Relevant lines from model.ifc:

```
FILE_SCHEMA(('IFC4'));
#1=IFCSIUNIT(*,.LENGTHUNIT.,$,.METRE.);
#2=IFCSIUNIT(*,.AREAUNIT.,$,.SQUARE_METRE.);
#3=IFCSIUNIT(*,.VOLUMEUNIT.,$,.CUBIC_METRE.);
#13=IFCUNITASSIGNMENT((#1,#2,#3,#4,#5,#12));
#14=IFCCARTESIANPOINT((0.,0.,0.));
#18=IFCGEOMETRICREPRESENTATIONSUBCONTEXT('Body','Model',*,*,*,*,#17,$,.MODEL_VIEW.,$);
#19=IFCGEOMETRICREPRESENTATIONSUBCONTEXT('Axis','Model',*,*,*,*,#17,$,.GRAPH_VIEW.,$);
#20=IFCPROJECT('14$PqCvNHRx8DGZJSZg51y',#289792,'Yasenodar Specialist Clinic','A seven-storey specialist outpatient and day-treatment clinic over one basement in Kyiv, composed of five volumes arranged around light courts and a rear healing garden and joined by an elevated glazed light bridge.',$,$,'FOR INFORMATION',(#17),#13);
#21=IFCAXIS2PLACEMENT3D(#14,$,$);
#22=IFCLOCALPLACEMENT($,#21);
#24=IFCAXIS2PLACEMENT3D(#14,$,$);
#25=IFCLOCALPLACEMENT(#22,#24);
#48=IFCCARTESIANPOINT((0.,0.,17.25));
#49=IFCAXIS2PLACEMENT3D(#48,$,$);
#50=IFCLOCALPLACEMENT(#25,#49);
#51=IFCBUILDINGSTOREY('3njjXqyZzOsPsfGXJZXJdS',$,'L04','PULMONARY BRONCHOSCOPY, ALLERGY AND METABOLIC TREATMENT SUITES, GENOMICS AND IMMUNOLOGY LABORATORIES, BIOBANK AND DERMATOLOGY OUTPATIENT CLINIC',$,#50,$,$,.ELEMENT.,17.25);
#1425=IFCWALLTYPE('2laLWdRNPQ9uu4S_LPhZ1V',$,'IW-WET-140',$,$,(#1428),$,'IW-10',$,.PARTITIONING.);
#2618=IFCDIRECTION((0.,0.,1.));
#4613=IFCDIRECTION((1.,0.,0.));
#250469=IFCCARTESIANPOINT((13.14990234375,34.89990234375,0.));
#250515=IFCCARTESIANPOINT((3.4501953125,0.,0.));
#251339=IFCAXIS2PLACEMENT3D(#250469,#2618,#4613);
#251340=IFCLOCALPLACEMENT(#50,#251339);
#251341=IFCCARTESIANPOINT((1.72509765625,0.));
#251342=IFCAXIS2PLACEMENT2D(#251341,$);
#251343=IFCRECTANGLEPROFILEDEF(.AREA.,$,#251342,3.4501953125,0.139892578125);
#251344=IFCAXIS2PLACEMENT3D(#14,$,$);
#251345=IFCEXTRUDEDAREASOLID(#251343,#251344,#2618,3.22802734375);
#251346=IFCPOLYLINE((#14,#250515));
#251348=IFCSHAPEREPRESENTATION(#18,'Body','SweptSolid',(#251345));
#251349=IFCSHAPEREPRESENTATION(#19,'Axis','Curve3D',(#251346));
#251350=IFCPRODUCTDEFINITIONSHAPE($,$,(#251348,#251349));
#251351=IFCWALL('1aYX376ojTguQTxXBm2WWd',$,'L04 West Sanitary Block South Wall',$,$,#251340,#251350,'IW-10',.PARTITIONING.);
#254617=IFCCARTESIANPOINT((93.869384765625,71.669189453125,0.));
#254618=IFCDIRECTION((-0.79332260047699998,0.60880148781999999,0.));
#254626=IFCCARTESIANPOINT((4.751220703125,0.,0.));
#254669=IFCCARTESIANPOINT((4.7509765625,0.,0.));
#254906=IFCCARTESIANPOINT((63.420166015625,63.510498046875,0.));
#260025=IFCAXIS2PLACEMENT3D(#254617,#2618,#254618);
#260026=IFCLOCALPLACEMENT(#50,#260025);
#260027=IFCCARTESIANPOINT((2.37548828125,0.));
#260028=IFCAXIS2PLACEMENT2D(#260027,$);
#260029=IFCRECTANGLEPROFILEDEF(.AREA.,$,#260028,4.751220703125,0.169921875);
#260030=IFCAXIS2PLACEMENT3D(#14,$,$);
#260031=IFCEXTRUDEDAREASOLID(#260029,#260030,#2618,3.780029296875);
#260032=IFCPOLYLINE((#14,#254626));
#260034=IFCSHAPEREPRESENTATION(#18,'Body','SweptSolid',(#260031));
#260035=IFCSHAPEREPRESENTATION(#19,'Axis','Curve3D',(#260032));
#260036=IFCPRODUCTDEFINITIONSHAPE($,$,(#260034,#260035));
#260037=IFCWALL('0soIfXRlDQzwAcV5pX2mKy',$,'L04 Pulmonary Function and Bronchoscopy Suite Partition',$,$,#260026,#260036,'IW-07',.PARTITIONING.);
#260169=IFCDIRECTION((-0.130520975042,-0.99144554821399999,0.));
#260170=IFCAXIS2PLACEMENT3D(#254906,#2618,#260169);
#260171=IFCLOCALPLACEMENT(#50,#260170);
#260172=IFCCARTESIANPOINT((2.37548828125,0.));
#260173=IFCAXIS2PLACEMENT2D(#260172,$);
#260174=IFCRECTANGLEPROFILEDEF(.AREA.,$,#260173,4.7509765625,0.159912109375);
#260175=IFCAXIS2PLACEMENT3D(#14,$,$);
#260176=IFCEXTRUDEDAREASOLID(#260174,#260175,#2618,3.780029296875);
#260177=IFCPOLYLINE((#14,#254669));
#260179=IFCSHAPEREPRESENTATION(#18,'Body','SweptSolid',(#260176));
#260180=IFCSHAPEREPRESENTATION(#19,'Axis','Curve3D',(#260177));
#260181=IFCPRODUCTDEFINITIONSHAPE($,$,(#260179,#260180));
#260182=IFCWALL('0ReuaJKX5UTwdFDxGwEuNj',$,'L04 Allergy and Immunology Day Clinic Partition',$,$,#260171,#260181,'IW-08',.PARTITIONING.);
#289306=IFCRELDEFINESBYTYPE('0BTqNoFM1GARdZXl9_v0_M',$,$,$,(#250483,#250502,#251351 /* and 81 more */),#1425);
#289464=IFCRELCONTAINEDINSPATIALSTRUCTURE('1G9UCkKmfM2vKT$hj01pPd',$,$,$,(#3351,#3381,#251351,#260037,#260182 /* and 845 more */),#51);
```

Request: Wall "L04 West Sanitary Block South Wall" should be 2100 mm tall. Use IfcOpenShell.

```python
import ifcopenshell
import ifcopenshell.geom
import ifcopenshell.util.representation
import ifcopenshell.util.shape
import ifcopenshell.util.unit

model = ifcopenshell.open("model.ifc")
unit_scale = ifcopenshell.util.unit.calculate_unit_scale(model)
settings = ifcopenshell.geom.settings()


def volume(element):
    """Net volume in cubic metres, openings subtracted."""
    shape = ifcopenshell.geom.create_shape(settings, element)
    return ifcopenshell.util.shape.get_volume(shape.geometry)


wall = model.by_guid("1aYX376ojTguQTxXBm2WWd")
before = volume(wall)

body = ifcopenshell.util.representation.get_representation(wall, "Model", "Body")
solid = body.Items[0]
old_height = solid.Depth
solid.Depth = 2.1 / unit_scale
after = volume(wall)

print(f"height {old_height:g} -> {solid.Depth:g}, volume {before:.3f} -> {after:.3f} m3")

model.write("model_rev.ifc")
```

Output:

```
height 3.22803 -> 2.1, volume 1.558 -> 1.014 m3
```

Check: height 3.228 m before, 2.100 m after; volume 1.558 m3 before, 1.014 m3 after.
